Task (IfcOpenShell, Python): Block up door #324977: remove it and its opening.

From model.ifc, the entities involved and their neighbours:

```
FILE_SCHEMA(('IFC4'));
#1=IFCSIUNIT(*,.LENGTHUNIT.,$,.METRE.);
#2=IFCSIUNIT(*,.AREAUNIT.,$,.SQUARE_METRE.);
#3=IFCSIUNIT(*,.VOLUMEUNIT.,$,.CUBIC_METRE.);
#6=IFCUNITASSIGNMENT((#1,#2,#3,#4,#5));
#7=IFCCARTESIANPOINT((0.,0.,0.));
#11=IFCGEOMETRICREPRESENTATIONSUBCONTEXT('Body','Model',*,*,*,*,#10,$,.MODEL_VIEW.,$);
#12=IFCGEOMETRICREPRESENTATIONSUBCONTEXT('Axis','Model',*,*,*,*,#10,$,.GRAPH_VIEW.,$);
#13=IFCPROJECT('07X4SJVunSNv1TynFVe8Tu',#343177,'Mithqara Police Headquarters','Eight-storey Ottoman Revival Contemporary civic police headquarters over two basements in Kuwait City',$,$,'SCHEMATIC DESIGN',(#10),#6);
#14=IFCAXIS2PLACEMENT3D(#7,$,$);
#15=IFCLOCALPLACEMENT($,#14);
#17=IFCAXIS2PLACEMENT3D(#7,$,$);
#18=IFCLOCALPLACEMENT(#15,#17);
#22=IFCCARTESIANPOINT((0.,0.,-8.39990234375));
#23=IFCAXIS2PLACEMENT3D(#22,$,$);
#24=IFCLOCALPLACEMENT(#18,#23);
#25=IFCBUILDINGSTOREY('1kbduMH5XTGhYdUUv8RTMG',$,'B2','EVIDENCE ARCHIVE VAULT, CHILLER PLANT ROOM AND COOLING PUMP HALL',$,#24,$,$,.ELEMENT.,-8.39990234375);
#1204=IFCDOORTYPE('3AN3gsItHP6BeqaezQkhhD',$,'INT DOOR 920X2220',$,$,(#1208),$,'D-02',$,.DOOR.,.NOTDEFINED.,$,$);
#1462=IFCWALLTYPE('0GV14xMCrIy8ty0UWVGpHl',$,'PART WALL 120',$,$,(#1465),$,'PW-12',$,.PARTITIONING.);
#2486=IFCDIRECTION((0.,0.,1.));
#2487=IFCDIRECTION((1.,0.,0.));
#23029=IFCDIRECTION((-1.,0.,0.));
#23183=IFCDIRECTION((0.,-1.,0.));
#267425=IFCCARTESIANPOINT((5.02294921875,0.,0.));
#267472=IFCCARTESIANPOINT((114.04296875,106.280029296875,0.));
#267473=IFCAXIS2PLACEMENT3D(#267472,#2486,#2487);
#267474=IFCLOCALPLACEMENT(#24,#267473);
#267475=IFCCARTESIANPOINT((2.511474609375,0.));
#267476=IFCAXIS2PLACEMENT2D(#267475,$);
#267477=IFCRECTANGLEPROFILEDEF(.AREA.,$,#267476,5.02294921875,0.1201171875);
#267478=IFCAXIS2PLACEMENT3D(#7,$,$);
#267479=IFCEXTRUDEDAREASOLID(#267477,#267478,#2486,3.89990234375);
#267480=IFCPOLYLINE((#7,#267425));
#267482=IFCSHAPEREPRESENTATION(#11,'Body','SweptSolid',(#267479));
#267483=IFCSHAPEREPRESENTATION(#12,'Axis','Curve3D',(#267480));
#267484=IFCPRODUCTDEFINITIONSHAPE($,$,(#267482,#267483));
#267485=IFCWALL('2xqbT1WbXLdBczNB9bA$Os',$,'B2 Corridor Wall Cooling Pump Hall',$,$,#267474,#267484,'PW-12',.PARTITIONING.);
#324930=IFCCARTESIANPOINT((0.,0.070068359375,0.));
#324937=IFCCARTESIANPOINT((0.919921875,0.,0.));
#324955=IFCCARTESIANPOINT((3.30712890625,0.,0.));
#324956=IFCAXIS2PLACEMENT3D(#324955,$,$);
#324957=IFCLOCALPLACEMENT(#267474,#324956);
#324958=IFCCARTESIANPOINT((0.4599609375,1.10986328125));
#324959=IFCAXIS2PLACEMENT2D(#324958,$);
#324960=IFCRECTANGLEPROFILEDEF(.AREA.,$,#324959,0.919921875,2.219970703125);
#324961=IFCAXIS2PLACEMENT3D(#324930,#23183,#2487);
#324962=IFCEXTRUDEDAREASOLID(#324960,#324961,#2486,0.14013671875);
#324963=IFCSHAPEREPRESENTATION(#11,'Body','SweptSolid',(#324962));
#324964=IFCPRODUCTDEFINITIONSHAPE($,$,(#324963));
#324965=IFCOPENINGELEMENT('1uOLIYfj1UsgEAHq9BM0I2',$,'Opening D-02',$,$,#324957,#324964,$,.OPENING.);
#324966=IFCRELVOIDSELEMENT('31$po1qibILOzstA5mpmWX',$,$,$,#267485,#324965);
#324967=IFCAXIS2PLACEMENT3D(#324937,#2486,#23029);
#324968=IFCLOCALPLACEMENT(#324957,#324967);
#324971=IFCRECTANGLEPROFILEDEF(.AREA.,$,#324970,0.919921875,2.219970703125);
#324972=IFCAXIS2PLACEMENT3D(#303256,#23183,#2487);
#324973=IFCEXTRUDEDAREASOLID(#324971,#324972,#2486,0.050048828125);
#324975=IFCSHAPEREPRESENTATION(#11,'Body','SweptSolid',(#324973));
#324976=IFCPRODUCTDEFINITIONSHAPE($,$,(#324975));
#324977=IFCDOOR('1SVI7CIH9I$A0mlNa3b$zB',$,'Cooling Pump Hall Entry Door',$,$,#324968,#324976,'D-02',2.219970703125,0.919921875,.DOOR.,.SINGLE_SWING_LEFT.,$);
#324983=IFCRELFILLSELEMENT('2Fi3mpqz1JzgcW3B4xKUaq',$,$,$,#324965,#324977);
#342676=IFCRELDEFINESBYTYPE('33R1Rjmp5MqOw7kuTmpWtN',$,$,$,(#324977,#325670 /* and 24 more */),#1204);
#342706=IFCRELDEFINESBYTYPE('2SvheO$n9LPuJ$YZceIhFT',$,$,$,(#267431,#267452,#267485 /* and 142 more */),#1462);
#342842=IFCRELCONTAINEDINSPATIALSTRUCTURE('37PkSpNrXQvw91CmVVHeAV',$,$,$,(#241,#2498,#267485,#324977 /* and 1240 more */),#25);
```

```python
import ifcopenshell
import ifcopenshell.api.feature
import ifcopenshell.api.root
import ifcopenshell.geom
import ifcopenshell.util.shape

model = ifcopenshell.open("model.ifc")
settings = ifcopenshell.geom.settings()


def volume(element):
    """Net volume in cubic metres, openings subtracted."""
    shape = ifcopenshell.geom.create_shape(settings, element)
    return ifcopenshell.util.shape.get_volume(shape.geometry)


door = model.by_id(324977)
opening = door.FillsVoids[0].RelatingOpeningElement
wall = opening.VoidsElements[0].RelatingBuildingElement
before = volume(wall)

ifcopenshell.api.root.remove_product(model, product=door)
ifcopenshell.api.feature.remove_feature(model, feature=opening)

after = volume(wall)

print(f"wall volume {before:.3f} -> {after:.3f} m3")

model.write("model_rev.ifc")
```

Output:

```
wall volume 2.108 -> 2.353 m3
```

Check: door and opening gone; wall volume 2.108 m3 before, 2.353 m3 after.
